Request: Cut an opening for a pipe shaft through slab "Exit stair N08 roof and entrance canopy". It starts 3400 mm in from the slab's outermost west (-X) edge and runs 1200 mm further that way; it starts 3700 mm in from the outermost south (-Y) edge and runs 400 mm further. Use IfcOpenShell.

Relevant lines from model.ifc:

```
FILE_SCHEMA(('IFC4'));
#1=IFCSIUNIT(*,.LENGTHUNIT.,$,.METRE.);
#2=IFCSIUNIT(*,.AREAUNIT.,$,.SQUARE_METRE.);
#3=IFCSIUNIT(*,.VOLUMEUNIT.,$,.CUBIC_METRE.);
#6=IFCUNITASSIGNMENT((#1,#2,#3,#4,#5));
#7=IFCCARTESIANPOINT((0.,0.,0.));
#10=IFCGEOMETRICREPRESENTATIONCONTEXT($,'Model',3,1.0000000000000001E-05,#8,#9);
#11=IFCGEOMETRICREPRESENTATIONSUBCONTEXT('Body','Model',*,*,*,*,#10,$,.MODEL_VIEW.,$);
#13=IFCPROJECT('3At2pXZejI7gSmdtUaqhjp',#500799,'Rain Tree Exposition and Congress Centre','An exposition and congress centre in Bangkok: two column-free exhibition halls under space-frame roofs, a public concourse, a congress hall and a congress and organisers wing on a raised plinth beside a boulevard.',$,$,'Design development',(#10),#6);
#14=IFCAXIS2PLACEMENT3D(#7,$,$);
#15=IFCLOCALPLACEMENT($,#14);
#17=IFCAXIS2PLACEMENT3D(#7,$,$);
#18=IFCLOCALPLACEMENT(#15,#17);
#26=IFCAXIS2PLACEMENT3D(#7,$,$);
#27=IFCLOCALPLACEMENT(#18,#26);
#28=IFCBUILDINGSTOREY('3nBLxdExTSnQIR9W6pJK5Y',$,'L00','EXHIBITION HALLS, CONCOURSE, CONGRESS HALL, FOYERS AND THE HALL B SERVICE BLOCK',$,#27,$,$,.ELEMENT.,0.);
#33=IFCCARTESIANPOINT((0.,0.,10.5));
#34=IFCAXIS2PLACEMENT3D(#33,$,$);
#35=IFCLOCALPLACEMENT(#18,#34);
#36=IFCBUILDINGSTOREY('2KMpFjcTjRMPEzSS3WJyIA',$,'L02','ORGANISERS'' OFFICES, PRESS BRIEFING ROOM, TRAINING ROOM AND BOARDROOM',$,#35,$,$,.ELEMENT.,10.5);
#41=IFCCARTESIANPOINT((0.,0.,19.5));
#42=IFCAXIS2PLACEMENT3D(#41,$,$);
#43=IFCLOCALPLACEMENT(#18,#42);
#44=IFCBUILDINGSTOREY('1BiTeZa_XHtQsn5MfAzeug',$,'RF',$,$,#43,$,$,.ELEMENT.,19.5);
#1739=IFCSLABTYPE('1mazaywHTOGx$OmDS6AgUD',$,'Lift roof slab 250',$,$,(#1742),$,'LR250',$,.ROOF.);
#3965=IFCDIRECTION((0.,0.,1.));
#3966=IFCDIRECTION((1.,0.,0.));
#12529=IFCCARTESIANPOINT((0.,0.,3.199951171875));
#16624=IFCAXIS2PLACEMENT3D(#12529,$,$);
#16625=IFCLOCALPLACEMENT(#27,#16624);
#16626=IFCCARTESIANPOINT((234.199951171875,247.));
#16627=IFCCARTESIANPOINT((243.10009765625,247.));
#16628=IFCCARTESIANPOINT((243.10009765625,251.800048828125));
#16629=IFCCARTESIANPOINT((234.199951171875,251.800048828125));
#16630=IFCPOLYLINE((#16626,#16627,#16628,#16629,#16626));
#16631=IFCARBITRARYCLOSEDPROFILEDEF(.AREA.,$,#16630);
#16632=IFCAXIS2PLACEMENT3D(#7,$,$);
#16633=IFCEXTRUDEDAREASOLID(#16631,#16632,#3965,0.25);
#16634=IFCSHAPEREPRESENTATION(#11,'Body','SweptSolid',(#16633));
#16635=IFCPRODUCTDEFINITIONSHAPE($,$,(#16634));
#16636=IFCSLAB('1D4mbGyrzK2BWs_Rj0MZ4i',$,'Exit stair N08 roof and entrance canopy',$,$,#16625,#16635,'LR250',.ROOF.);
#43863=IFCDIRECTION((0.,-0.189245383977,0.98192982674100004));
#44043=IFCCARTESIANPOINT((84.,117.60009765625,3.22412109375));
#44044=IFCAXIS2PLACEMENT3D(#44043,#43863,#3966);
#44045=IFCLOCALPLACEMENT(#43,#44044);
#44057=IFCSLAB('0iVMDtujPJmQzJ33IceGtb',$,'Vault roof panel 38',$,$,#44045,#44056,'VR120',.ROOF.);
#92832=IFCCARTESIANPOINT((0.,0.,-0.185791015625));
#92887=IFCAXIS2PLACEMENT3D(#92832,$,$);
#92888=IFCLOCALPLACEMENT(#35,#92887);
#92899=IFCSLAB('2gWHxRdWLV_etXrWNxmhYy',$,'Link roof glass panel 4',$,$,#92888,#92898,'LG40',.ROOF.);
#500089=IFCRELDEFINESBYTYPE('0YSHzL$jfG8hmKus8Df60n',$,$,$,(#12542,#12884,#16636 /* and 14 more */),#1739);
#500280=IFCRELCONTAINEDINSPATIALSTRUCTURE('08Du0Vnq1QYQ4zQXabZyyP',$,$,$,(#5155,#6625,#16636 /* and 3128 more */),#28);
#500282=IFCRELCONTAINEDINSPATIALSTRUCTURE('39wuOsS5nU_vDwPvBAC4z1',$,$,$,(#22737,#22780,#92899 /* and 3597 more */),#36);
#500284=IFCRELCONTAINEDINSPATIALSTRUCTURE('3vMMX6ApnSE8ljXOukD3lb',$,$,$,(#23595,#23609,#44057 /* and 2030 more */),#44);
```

```python
import numpy as np
import ifcopenshell
import ifcopenshell.api.feature
import ifcopenshell.api.geometry
import ifcopenshell.api.root
import ifcopenshell.geom
import ifcopenshell.util.placement
import ifcopenshell.util.representation
import ifcopenshell.util.shape
import ifcopenshell.util.unit

model = ifcopenshell.open("model.ifc")
unit_scale = ifcopenshell.util.unit.calculate_unit_scale(model)
settings = ifcopenshell.geom.settings()


def volume(element):
    """Net volume in cubic metres, openings subtracted."""
    shape = ifcopenshell.geom.create_shape(settings, element)
    return ifcopenshell.util.shape.get_volume(shape.geometry)


slab = model.by_guid("1D4mbGyrzK2BWs_Rj0MZ4i")
before = volume(slab)

# Extent in the slab's own axes, in metres. The edges named are its -X and -Y sides.
slab_shape = ifcopenshell.geom.create_shape(settings, slab)
vertices = ifcopenshell.util.shape.get_vertices(slab_shape.geometry)
x_min, y_min, bottom = vertices.min(axis=0)
top = vertices[:, 2].max()

opening = ifcopenshell.api.root.create_entity(model, ifc_class="IfcOpeningElement", name="Pipe shaft opening", predefined_type="OPENING")
context = ifcopenshell.util.representation.get_context(model, "Model", "Body", "MODEL_VIEW")
width, depth = 1.2, 0.4
outline = [(0.0, 0.0), (width, 0.0), (width, depth), (0.0, depth), (0.0, 0.0)]
# Overshoot both faces by 50 mm so the cut is clean.
shape = ifcopenshell.api.geometry.add_slab_representation(
    model, context=context, depth=top - bottom + 0.1, polyline=outline
)
ifcopenshell.api.geometry.assign_representation(model, product=opening, representation=shape)

matrix = ifcopenshell.util.placement.get_local_placement(slab.ObjectPlacement)
matrix[:, 3] = matrix @ np.append(np.array([x_min + 3.4, y_min + 3.7, bottom - 0.05]) / unit_scale, 1.0)
ifcopenshell.api.geometry.edit_object_placement(model, product=opening, matrix=matrix, is_si=False)
ifcopenshell.api.feature.add_feature(model, feature=opening, element=slab)

after = volume(slab)

print(f"slab volume {before:.3f} -> {after:.3f} m3")

model.write("model_edited.ifc")
```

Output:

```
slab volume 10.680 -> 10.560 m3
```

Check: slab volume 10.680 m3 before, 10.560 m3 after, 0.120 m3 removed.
